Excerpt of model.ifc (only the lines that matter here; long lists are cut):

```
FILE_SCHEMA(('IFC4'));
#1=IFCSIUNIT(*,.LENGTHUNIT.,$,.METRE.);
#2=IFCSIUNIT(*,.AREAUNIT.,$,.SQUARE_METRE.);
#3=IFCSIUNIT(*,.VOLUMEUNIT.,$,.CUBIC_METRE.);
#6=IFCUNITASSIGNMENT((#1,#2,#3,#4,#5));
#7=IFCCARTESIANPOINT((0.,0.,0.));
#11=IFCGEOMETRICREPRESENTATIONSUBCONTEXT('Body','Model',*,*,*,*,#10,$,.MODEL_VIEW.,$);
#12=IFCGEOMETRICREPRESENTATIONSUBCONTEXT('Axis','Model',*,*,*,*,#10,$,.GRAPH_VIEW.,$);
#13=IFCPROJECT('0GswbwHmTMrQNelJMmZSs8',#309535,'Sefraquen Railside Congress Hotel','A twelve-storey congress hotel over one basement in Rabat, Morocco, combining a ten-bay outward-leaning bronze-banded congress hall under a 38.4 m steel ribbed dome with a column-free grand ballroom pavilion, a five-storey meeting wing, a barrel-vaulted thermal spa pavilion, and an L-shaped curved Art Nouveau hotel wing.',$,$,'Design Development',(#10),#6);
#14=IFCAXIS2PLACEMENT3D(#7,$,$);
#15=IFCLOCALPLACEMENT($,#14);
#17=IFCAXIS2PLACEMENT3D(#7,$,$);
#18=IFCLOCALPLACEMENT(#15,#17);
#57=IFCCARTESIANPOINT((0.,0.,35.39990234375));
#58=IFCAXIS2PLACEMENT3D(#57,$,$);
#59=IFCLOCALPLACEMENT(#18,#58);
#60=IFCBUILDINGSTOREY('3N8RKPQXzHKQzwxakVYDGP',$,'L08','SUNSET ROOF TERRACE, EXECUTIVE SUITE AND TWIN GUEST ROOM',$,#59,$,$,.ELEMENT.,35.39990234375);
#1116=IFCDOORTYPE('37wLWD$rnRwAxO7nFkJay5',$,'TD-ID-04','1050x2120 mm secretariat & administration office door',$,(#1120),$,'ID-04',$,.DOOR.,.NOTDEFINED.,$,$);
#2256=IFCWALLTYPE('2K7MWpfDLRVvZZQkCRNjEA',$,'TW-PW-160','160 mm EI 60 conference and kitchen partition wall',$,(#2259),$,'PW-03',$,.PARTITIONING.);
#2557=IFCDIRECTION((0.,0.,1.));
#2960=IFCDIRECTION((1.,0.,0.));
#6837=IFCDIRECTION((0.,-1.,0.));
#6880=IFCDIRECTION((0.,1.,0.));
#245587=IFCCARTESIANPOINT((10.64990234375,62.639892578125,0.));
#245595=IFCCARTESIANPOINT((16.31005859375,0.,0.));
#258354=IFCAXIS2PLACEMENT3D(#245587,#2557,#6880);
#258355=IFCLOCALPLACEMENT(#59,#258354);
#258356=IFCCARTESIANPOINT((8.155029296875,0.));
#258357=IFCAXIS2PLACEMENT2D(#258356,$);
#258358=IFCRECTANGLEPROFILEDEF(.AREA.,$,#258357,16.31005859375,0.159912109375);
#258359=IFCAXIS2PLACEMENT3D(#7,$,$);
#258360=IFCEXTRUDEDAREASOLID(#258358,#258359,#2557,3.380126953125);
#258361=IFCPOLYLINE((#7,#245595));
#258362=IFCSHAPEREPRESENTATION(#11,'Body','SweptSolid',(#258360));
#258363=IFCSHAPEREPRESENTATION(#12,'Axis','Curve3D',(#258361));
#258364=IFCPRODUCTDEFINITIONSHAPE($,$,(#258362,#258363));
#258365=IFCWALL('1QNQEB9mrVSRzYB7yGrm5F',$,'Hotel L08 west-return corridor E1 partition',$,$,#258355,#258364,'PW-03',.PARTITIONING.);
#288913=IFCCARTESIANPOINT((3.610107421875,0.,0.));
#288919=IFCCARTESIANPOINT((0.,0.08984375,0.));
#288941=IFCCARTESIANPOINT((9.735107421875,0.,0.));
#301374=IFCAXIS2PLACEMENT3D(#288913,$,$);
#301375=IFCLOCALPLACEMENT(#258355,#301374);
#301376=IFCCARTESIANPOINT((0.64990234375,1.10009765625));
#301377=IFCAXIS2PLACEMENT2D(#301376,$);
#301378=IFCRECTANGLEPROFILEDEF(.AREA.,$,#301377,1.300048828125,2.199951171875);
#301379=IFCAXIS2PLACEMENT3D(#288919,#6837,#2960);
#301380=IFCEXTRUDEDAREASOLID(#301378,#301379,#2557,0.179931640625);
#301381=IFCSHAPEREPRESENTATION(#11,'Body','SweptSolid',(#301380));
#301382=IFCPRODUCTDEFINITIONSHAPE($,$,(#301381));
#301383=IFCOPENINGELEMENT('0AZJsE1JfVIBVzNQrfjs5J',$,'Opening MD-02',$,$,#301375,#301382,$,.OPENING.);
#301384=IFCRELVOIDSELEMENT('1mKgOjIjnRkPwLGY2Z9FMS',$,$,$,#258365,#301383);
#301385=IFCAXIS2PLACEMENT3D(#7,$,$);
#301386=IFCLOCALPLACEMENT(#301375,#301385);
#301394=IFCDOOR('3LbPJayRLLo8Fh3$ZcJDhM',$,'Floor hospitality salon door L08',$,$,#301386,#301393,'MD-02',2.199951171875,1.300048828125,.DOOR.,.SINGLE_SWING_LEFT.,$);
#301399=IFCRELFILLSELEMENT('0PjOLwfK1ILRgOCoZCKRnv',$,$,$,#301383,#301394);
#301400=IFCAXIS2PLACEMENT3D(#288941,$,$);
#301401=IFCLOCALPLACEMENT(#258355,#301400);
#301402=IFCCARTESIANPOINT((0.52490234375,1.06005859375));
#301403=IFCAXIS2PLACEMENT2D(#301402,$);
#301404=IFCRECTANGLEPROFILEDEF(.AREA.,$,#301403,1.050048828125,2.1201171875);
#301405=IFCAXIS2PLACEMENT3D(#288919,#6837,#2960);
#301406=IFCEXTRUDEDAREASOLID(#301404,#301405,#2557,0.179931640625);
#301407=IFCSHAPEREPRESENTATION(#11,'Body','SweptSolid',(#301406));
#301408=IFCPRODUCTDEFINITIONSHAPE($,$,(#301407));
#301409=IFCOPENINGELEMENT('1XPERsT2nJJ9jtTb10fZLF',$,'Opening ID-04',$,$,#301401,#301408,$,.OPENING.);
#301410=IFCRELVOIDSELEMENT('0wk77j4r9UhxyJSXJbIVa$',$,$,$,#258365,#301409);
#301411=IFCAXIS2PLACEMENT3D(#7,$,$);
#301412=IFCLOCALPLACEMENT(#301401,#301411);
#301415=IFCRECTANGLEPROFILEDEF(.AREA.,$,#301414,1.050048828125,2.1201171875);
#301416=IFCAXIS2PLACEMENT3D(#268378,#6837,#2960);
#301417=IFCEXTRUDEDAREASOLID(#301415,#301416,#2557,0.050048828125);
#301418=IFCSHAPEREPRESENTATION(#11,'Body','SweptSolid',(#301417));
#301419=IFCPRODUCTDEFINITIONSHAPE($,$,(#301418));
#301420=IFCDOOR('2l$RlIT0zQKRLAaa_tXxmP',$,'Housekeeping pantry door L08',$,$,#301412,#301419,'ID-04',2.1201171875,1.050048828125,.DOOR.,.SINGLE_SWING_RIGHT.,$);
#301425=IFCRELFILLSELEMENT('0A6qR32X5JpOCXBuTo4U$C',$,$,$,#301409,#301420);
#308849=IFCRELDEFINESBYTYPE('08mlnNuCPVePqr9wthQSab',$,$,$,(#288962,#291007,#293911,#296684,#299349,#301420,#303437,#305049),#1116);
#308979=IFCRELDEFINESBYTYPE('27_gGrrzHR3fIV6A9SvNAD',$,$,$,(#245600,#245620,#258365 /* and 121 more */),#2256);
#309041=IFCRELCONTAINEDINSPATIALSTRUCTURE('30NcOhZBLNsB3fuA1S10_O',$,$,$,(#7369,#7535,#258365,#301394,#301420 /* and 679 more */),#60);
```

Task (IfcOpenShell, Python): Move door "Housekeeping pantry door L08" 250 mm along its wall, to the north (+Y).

```python
import ifcopenshell
import ifcopenshell.api.geometry
import ifcopenshell.util.placement

model = ifcopenshell.open("model.ifc")

door = model.by_guid("2l$RlIT0zQKRLAaa_tXxmP")
opening = door.FillsVoids[0].RelatingOpeningElement
wall = opening.VoidsElements[0].RelatingBuildingElement

wall_matrix = ifcopenshell.util.placement.get_local_placement(wall.ObjectPlacement)
shift = wall_matrix[:3, 0] * 0.25
before = ifcopenshell.util.placement.get_local_placement(door.ObjectPlacement)[:3, 3].copy()

# The door is placed relative to its opening, so it follows when the opening moves.
matrix = ifcopenshell.util.placement.get_local_placement(opening.ObjectPlacement)
matrix[:3, 3] += shift
ifcopenshell.api.geometry.edit_object_placement(
    model, product=opening, matrix=matrix, is_si=False, should_transform_children=True
)

after = ifcopenshell.util.placement.get_local_placement(door.ObjectPlacement)[:3, 3]
print("door moved by", (after - before).round(3) + 0.0)

model.write("model-out.ifc")
```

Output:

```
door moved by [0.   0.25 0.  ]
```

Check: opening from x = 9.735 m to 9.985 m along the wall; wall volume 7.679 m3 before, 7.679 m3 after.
